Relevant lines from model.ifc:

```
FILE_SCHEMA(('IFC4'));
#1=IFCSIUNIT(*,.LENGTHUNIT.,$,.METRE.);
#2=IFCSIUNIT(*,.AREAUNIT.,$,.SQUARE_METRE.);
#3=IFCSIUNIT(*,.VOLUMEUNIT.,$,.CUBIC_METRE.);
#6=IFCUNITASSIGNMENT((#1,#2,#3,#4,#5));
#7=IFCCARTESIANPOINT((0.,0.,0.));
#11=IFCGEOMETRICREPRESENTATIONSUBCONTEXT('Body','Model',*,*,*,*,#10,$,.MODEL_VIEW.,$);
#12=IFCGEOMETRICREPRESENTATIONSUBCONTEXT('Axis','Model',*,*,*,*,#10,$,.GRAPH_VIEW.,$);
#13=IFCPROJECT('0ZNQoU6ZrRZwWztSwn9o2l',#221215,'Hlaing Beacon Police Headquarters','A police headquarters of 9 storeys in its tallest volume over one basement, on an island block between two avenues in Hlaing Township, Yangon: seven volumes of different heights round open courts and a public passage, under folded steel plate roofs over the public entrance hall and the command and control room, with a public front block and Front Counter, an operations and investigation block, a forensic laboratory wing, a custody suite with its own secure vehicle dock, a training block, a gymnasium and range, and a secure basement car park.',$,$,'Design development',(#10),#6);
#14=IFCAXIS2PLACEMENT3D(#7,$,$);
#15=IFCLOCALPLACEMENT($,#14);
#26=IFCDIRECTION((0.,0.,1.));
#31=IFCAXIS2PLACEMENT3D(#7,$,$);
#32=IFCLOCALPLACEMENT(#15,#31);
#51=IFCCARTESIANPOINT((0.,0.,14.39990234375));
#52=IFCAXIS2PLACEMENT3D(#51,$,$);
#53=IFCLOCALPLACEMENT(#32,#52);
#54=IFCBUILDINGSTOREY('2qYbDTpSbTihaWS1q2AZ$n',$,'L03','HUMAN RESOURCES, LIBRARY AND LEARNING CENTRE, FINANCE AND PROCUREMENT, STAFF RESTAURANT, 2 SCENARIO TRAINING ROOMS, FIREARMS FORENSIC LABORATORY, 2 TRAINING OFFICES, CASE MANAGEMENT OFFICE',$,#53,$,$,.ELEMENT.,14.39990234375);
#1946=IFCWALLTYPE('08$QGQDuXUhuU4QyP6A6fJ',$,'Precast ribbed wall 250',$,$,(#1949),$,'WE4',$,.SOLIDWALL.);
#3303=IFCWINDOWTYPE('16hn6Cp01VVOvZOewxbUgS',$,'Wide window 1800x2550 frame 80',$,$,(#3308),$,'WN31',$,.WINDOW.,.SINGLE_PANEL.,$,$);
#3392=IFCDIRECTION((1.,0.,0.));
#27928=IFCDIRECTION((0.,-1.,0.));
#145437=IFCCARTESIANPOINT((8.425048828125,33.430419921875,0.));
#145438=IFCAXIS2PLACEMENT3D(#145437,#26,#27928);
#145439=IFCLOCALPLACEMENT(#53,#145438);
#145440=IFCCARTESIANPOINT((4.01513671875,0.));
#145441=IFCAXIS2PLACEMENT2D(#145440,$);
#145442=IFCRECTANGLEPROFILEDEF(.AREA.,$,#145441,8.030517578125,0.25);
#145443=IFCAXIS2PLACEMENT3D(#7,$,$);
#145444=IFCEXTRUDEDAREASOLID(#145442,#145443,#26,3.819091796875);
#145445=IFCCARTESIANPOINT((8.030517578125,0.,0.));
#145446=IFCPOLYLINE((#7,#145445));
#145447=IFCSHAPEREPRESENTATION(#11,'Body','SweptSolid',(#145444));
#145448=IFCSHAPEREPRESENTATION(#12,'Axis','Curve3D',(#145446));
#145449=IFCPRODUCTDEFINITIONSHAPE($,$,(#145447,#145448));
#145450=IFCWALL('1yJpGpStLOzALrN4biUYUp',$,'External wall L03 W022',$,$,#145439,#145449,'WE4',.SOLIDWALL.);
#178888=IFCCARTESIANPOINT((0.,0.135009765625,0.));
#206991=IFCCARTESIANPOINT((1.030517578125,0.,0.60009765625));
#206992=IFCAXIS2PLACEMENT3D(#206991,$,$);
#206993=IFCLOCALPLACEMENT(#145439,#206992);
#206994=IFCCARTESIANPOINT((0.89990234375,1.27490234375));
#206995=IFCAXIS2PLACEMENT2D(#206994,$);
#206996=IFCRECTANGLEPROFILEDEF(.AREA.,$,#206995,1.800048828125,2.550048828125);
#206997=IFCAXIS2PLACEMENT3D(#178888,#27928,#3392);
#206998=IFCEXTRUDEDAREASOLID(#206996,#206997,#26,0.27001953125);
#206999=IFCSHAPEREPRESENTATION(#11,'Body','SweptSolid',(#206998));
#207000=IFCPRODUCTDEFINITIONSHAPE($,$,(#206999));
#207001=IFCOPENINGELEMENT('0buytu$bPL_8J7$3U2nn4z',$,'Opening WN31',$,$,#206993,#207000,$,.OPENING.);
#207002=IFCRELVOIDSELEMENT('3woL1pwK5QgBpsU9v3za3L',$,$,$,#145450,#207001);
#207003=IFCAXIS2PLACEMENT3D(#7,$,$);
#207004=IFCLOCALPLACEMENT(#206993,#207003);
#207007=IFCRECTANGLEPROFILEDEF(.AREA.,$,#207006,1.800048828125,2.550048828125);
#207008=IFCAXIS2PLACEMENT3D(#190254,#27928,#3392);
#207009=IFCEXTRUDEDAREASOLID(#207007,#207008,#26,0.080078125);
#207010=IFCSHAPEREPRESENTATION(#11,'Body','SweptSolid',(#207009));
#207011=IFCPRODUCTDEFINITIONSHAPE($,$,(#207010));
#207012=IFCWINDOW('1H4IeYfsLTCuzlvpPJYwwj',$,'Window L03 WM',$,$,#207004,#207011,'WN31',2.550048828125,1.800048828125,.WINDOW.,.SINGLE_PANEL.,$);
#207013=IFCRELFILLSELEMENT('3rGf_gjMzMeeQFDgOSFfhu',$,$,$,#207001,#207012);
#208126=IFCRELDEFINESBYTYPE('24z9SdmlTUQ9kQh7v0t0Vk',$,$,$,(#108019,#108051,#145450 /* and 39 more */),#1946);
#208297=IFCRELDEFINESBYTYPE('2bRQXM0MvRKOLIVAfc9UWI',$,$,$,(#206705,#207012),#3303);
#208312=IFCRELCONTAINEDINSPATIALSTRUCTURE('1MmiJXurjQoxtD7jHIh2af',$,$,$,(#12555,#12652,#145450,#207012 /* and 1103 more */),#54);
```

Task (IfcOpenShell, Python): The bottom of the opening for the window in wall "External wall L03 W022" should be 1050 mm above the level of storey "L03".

```python
import numpy as np
import ifcopenshell
import ifcopenshell.api.geometry
import ifcopenshell.geom
import ifcopenshell.util.element
import ifcopenshell.util.placement
import ifcopenshell.util.shape
import ifcopenshell.util.unit

model = ifcopenshell.open("model.ifc")
unit_scale = ifcopenshell.util.unit.calculate_unit_scale(model)

window = model.by_guid("1H4IeYfsLTCuzlvpPJYwwj")
opening = window.FillsVoids[0].RelatingOpeningElement
storey = ifcopenshell.util.element.get_container(window, ifc_class="IfcBuildingStorey")
level = ifcopenshell.util.placement.get_local_placement(storey.ObjectPlacement)[2, 3]

# The opening's origin need not be at the sill, so measure its lowest point.
shape = ifcopenshell.geom.create_shape(ifcopenshell.geom.settings(), opening)
bottom = ifcopenshell.util.shape.get_shape_bottom_elevation(shape, shape.geometry) / unit_scale
dz = level + 1.05 / unit_scale - bottom

shift = np.array([0.0, 0.0, dz])
# The window is placed relative to its opening, so it follows when the opening moves.
matrix = ifcopenshell.util.placement.get_local_placement(opening.ObjectPlacement)
matrix[:3, 3] += shift
ifcopenshell.api.geometry.edit_object_placement(
    model, product=opening, matrix=matrix, is_si=False, should_transform_children=True
)

print(f"moved by {dz * unit_scale:+.3f} m")

model.write("model-out.ifc")
```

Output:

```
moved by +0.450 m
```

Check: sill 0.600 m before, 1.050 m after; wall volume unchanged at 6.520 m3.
